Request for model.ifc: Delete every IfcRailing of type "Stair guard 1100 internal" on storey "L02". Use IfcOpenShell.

First a look at what the model holds.

```python
import ifcopenshell
import ifcopenshell.util.element

model = ifcopenshell.open("model.ifc")
print(model.schema)
storey = next(s for s in model.by_type("IfcBuildingStorey") if s.Name == "L02")
railings = [e for e in ifcopenshell.util.element.get_decomposition(storey) if e.is_a("IfcRailing")]
seen = {}
for e in railings:
    element_type = ifcopenshell.util.element.get_type(e)
    name = element_type.Name if element_type not in (None, e) else None
    seen[name] = seen.get(name, 0) + 1
for name, count in sorted(seen.items(), key=str):
    print(count, "x", name)
```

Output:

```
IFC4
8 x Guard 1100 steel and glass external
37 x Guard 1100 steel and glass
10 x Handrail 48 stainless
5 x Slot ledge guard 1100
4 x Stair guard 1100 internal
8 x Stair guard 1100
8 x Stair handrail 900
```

```python
import ifcopenshell
import ifcopenshell.api.root
import ifcopenshell.util.element

model = ifcopenshell.open("model.ifc")

storey = next(s for s in model.by_type("IfcBuildingStorey") if s.Name == "L02")
railings = [e for e in ifcopenshell.util.element.get_decomposition(storey) if e.is_a("IfcRailing")]
targets = [e for e in railings if (t := ifcopenshell.util.element.get_type(e)) not in (None, e) and t.Name == "Stair guard 1100 internal"]

for e in targets:
    ifcopenshell.api.root.remove_product(model, product=e)
print(len(targets), "removed")

model.write("model_edited.ifc")
```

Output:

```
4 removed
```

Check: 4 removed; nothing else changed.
